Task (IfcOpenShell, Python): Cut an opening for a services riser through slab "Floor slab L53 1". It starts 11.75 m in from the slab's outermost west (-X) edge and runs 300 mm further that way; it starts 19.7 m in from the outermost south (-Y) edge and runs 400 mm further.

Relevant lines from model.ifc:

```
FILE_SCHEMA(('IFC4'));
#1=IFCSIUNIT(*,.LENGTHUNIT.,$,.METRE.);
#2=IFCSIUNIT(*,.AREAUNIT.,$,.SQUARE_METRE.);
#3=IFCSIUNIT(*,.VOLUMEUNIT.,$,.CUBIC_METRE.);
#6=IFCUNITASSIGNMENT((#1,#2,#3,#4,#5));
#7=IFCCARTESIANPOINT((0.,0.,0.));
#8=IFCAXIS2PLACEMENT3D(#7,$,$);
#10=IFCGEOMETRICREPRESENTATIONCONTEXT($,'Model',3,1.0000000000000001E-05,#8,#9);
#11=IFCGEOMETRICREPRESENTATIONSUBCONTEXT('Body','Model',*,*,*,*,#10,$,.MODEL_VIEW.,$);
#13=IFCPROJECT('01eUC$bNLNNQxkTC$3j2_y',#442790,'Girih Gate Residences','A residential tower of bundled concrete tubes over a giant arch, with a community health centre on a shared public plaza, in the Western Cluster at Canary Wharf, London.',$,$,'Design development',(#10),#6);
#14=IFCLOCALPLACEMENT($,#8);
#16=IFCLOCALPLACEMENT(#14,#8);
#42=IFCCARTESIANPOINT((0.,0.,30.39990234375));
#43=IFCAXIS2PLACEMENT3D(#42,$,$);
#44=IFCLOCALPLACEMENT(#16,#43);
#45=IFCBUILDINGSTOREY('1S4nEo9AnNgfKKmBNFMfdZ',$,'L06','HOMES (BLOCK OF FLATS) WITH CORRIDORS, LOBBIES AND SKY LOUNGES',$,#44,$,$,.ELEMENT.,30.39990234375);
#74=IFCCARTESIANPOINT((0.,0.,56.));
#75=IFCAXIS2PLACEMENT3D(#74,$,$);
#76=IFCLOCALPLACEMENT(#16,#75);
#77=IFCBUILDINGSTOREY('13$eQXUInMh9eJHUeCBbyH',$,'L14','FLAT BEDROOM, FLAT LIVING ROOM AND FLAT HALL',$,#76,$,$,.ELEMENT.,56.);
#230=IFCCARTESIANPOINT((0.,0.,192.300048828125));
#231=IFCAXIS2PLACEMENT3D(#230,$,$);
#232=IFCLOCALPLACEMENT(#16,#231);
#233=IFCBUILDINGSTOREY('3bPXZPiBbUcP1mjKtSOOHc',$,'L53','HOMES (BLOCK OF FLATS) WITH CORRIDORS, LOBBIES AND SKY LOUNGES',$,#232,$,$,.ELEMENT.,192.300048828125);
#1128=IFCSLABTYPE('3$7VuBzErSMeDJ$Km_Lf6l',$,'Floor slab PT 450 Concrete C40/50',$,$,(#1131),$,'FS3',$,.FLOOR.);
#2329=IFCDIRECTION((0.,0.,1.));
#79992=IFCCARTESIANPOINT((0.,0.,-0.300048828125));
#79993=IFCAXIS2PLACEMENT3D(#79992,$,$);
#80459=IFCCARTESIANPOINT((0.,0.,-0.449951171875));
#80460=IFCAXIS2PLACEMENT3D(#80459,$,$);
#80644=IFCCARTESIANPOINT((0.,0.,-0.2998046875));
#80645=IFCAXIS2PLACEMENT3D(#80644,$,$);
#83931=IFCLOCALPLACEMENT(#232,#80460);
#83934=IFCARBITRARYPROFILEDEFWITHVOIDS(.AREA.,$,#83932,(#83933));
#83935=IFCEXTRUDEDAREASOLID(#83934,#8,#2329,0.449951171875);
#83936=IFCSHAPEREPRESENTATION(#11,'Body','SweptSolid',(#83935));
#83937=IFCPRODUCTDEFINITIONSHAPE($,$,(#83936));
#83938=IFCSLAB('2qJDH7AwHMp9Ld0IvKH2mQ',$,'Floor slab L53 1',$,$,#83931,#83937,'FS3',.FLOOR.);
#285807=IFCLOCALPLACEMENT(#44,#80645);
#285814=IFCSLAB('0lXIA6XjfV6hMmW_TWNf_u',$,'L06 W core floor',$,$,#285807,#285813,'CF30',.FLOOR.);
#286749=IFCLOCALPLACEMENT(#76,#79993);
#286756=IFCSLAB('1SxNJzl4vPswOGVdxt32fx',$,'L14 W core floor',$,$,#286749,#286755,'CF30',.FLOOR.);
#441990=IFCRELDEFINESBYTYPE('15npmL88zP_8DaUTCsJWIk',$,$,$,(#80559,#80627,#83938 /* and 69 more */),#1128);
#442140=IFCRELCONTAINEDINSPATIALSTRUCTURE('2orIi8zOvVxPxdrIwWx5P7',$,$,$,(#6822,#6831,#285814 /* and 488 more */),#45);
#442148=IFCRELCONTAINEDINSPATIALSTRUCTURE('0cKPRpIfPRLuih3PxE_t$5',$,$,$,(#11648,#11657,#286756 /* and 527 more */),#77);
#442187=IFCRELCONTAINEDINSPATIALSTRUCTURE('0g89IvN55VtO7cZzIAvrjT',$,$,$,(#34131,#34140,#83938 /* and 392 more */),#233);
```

```python
import numpy as np
import ifcopenshell
import ifcopenshell.api.feature
import ifcopenshell.api.geometry
import ifcopenshell.api.root
import ifcopenshell.geom
import ifcopenshell.util.placement
import ifcopenshell.util.representation
import ifcopenshell.util.shape
import ifcopenshell.util.unit

model = ifcopenshell.open("model.ifc")
unit_scale = ifcopenshell.util.unit.calculate_unit_scale(model)
settings = ifcopenshell.geom.settings()


def volume(element):
    """Net volume in cubic metres, openings subtracted."""
    shape = ifcopenshell.geom.create_shape(settings, element)
    return ifcopenshell.util.shape.get_volume(shape.geometry)


slab = model.by_guid("2qJDH7AwHMp9Ld0IvKH2mQ")
before = volume(slab)

# Extent in the slab's own axes, in metres. The edges named are its -X and -Y sides.
slab_shape = ifcopenshell.geom.create_shape(settings, slab)
vertices = ifcopenshell.util.shape.get_vertices(slab_shape.geometry)
x_min, y_min, bottom = vertices.min(axis=0)
top = vertices[:, 2].max()

opening = ifcopenshell.api.root.create_entity(model, ifc_class="IfcOpeningElement", name="Services riser opening", predefined_type="OPENING")
context = ifcopenshell.util.representation.get_context(model, "Model", "Body", "MODEL_VIEW")
width, depth = 0.3, 0.4
outline = [(0.0, 0.0), (width, 0.0), (width, depth), (0.0, depth), (0.0, 0.0)]
# Overshoot both faces by 50 mm so the cut is clean.
shape = ifcopenshell.api.geometry.add_slab_representation(
    model, context=context, depth=top - bottom + 0.1, polyline=outline
)
ifcopenshell.api.geometry.assign_representation(model, product=opening, representation=shape)

matrix = ifcopenshell.util.placement.get_local_placement(slab.ObjectPlacement)
matrix[:, 3] = matrix @ np.append(np.array([x_min + 11.75, y_min + 19.7, bottom - 0.05]) / unit_scale, 1.0)
ifcopenshell.api.geometry.edit_object_placement(model, product=opening, matrix=matrix, is_si=False)
ifcopenshell.api.feature.add_feature(model, feature=opening, element=slab)

after = volume(slab)

print(f"slab volume {before:.3f} -> {after:.3f} m3")

model.write("model_updated.ifc")
```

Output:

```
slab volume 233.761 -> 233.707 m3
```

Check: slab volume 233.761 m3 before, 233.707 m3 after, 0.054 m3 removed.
